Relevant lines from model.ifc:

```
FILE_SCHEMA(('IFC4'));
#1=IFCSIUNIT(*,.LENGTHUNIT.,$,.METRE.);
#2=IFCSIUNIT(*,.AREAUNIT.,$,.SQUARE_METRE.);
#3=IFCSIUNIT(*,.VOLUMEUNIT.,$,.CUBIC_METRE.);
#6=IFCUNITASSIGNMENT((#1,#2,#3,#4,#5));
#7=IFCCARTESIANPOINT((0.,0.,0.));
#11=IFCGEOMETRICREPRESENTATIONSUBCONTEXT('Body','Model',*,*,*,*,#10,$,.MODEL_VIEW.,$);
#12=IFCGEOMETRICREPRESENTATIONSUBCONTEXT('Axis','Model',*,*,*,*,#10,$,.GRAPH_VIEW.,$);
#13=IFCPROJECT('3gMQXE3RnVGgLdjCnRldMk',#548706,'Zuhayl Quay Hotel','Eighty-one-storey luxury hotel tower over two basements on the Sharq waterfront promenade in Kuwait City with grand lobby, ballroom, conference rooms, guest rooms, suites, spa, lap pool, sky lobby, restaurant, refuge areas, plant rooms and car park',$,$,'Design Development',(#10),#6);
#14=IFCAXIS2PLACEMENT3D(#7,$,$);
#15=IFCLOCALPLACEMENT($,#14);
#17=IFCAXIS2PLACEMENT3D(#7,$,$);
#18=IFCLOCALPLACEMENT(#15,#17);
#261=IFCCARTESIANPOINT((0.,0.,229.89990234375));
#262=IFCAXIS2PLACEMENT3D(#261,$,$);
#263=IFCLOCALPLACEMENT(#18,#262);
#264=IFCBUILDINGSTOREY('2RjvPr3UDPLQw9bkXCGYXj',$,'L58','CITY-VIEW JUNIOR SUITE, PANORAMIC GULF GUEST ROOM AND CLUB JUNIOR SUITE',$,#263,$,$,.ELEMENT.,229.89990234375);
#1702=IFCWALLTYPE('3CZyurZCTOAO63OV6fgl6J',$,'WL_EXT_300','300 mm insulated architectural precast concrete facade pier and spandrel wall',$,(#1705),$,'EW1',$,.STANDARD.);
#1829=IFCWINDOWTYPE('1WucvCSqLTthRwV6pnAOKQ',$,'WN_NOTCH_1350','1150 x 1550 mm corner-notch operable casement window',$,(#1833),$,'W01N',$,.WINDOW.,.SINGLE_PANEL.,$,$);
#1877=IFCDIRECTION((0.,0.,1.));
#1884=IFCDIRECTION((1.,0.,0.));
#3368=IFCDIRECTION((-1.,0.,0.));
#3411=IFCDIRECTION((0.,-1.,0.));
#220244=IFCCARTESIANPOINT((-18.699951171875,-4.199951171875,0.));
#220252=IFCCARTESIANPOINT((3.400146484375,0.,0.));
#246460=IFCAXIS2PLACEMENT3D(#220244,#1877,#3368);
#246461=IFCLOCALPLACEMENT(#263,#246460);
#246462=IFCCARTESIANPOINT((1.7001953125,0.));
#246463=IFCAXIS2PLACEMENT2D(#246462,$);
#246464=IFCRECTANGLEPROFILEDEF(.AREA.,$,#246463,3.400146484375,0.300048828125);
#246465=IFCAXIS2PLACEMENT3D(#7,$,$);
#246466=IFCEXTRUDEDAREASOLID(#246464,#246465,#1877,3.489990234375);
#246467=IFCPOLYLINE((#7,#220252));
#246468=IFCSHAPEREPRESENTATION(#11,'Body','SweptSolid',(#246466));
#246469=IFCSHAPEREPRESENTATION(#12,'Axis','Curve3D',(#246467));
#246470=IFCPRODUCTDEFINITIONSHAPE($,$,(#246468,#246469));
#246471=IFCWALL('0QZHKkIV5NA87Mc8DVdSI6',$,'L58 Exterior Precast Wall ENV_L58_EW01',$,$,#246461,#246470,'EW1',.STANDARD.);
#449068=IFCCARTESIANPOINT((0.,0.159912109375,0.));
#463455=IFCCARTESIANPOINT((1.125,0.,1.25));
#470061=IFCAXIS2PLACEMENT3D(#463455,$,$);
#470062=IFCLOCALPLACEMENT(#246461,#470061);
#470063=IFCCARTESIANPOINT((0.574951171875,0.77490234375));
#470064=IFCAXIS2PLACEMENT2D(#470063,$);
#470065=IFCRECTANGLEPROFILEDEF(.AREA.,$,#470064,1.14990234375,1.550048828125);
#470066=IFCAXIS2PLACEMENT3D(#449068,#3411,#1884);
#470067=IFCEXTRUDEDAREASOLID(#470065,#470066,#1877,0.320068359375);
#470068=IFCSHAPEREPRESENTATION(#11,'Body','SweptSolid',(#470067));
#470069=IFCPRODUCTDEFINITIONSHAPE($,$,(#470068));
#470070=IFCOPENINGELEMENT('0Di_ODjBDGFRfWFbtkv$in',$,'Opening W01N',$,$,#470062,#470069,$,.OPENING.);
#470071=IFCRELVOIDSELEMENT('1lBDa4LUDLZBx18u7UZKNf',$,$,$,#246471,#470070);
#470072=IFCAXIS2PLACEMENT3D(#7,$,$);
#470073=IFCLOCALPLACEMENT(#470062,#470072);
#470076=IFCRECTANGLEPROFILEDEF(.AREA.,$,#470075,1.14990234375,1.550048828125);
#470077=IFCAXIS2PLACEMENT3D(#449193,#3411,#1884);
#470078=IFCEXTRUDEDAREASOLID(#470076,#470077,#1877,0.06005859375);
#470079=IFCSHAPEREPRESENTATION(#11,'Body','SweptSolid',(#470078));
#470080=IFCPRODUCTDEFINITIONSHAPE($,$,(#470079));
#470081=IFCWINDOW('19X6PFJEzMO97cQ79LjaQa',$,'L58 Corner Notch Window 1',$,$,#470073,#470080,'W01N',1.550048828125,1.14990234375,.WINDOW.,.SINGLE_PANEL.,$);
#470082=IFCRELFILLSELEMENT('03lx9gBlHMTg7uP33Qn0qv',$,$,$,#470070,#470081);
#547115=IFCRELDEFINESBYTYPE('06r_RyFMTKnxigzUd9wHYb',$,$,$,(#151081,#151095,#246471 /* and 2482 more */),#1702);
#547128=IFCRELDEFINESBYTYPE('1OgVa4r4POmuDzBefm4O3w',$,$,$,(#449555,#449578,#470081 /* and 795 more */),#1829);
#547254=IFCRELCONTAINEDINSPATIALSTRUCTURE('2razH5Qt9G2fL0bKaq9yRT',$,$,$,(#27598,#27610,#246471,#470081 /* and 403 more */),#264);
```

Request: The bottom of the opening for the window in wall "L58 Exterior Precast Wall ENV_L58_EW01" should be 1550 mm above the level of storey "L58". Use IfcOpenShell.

```python
import numpy as np
import ifcopenshell
import ifcopenshell.api.geometry
import ifcopenshell.geom
import ifcopenshell.util.element
import ifcopenshell.util.placement
import ifcopenshell.util.shape
import ifcopenshell.util.unit

model = ifcopenshell.open("model.ifc")
unit_scale = ifcopenshell.util.unit.calculate_unit_scale(model)

window = model.by_id(470081)
opening = window.FillsVoids[0].RelatingOpeningElement
storey = ifcopenshell.util.element.get_container(window, ifc_class="IfcBuildingStorey")
level = ifcopenshell.util.placement.get_local_placement(storey.ObjectPlacement)[2, 3]

# The opening's origin need not be at the sill, so measure its lowest point.
shape = ifcopenshell.geom.create_shape(ifcopenshell.geom.settings(), opening)
bottom = ifcopenshell.util.shape.get_shape_bottom_elevation(shape, shape.geometry) / unit_scale
dz = level + 1.55 / unit_scale - bottom

shift = np.array([0.0, 0.0, dz])
# The window is placed relative to its opening, so it follows when the opening moves.
matrix = ifcopenshell.util.placement.get_local_placement(opening.ObjectPlacement)
matrix[:3, 3] += shift
ifcopenshell.api.geometry.edit_object_placement(
    model, product=opening, matrix=matrix, is_si=False, should_transform_children=True
)

print(f"moved by {dz * unit_scale:+.3f} m")

model.write("model_v2.ifc")
```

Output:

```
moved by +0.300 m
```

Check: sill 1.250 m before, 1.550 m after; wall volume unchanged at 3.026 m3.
